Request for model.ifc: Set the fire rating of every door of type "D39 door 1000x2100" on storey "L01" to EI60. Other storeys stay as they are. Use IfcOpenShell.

First a look at what the model holds.

```python
import ifcopenshell
import ifcopenshell.util.element

model = ifcopenshell.open("model.ifc")
print(model.schema)
storey = next(s for s in model.by_type("IfcBuildingStorey") if s.Name == "L01")
doors = [e for e in ifcopenshell.util.element.get_decomposition(storey) if e.is_a("IfcDoor")]
seen = {}
for e in doors:
    element_type = ifcopenshell.util.element.get_type(e)
    key = (element_type.Name if element_type != e and element_type else None, ifcopenshell.util.element.get_pset(e, "Pset_DoorCommon", "FireRating"))
    seen[key] = seen.get(key, 0) + 1
for (name, value), count in sorted(seen.items(), key=str):
    print(count, "x", name, "|", value)
```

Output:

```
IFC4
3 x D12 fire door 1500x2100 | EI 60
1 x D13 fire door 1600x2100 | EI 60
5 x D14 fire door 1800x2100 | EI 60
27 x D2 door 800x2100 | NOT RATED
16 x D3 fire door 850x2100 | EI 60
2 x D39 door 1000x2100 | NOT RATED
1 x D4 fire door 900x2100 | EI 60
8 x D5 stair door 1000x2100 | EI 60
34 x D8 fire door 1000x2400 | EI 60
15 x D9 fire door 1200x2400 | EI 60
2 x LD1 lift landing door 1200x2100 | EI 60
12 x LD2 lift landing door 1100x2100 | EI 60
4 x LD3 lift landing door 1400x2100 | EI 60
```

```python
import ifcopenshell
import ifcopenshell.api.pset
import ifcopenshell.util.element

model = ifcopenshell.open("model.ifc")

storey = next(s for s in model.by_type("IfcBuildingStorey") if s.Name == "L01")
doors = [e for e in ifcopenshell.util.element.get_decomposition(storey) if e.is_a("IfcDoor")]

count = 0
for e in doors:
    element_type = ifcopenshell.util.element.get_type(e)
    if element_type in (None, e) or element_type.Name != "D39 door 1000x2100":
        continue
    # add_pset returns the element's existing set when there is one.
    pset = ifcopenshell.api.pset.add_pset(model, product=e, name="Pset_DoorCommon")
    ifcopenshell.api.pset.edit_pset(model, pset=pset, properties={"FireRating": "EI60"})
    count += 1

print(count, "doors updated")

model.write("model_rev.ifc")
```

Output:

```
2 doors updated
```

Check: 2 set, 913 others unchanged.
